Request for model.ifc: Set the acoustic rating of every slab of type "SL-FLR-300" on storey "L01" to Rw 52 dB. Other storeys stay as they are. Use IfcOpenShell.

First a look at what the model holds.

```python
import ifcopenshell
import ifcopenshell.util.element

model = ifcopenshell.open("model.ifc")
print(model.schema)
storey = next(s for s in model.by_type("IfcBuildingStorey") if s.Name == "L01")
slabs = [e for e in ifcopenshell.util.element.get_decomposition(storey) if e.is_a("IfcSlab")]
seen = {}
for e in slabs:
    element_type = ifcopenshell.util.element.get_type(e)
    key = (element_type.Name if element_type != e and element_type else None, ifcopenshell.util.element.get_pset(e, "Pset_SlabCommon", "AcousticRating"))
    seen[key] = seen.get(key, 0) + 1
for (name, value), count in sorted(seen.items(), key=str):
    print(count, "x", name, "|", value)
```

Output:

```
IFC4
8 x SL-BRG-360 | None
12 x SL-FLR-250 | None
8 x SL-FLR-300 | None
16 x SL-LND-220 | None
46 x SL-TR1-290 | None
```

```python
import ifcopenshell
import ifcopenshell.api.pset
import ifcopenshell.util.element

model = ifcopenshell.open("model.ifc")

storey = next(s for s in model.by_type("IfcBuildingStorey") if s.Name == "L01")
slabs = [e for e in ifcopenshell.util.element.get_decomposition(storey) if e.is_a("IfcSlab")]

count = 0
for e in slabs:
    element_type = ifcopenshell.util.element.get_type(e)
    if element_type in (None, e) or element_type.Name != "SL-FLR-300":
        continue
    # add_pset returns the element's existing set when there is one.
    pset = ifcopenshell.api.pset.add_pset(model, product=e, name="Pset_SlabCommon")
    ifcopenshell.api.pset.edit_pset(model, pset=pset, properties={"AcousticRating": "Rw 52 dB"})
    count += 1

print(count, "slabs updated")

model.write("model_updated.ifc")
```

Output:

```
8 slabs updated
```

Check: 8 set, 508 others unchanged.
